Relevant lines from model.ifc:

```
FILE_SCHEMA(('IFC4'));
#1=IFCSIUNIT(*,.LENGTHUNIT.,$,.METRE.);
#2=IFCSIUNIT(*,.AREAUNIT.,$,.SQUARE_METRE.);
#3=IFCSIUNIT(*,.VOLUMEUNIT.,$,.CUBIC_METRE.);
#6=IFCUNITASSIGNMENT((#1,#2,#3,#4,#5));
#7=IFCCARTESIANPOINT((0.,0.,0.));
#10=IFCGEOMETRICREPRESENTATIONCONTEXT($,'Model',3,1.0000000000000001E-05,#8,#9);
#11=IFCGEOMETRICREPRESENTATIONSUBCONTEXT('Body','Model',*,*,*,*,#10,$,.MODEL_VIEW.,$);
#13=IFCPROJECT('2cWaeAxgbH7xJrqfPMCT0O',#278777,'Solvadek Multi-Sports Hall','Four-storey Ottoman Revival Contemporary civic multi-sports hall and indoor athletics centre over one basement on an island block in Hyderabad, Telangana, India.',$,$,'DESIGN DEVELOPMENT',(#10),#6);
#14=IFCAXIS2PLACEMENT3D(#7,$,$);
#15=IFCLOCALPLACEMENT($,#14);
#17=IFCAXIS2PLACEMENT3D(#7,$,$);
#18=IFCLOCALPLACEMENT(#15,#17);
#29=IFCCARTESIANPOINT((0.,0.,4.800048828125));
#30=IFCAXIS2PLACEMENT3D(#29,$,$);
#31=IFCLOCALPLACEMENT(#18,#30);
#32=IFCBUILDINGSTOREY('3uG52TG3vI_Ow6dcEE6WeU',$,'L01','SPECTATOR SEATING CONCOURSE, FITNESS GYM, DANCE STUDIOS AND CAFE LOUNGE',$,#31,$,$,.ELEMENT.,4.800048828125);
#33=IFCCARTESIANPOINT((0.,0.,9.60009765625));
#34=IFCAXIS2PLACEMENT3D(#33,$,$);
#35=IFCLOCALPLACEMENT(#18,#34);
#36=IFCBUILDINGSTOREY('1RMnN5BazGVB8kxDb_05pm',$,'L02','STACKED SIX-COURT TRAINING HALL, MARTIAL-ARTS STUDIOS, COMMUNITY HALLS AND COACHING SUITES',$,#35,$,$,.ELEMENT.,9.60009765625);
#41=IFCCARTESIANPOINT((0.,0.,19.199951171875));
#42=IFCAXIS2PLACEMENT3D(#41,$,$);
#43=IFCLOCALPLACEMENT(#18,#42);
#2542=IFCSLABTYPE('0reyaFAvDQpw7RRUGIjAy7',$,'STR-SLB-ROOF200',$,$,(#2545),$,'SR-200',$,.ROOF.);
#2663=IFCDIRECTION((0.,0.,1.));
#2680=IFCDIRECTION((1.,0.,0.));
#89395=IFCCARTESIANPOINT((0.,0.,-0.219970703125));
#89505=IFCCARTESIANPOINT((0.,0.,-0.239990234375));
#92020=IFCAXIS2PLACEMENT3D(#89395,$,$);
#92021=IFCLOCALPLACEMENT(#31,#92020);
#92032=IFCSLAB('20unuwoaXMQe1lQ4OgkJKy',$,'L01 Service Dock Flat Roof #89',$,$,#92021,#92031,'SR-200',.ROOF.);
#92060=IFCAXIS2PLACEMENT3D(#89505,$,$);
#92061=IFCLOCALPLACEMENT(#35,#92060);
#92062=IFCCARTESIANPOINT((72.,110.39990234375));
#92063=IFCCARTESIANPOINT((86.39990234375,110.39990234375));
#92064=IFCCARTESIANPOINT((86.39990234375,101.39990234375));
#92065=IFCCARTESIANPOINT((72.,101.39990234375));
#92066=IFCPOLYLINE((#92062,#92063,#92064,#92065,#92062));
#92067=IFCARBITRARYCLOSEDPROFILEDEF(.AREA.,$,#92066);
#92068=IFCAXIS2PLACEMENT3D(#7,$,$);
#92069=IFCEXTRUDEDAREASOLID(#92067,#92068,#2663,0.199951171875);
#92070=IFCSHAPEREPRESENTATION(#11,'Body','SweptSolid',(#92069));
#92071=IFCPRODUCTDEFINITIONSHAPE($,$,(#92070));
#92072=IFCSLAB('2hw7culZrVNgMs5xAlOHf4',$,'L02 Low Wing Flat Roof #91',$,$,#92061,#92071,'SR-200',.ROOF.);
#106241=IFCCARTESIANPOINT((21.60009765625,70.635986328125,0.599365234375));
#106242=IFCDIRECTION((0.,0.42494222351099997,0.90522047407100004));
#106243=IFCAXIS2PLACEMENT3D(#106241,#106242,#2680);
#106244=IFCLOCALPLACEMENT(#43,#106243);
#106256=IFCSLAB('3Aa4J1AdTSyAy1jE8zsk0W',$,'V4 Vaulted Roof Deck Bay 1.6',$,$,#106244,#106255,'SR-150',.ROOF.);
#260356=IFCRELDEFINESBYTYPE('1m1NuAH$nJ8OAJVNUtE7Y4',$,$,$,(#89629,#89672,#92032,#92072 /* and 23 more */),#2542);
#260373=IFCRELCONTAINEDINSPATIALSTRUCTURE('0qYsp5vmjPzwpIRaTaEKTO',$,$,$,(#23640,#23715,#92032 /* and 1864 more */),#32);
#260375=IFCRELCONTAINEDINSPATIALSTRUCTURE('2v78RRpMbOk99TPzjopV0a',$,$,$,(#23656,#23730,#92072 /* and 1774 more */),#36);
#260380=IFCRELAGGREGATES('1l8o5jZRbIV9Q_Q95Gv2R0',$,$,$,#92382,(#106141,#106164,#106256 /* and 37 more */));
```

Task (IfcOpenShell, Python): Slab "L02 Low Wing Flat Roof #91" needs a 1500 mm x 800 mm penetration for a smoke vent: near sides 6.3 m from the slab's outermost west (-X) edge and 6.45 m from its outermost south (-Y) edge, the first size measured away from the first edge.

```python
import numpy as np
import ifcopenshell
import ifcopenshell.api.feature
import ifcopenshell.api.geometry
import ifcopenshell.api.root
import ifcopenshell.geom
import ifcopenshell.util.placement
import ifcopenshell.util.representation
import ifcopenshell.util.shape
import ifcopenshell.util.unit

model = ifcopenshell.open("model.ifc")
unit_scale = ifcopenshell.util.unit.calculate_unit_scale(model)
settings = ifcopenshell.geom.settings()


def volume(element):
    """Net volume in cubic metres, openings subtracted."""
    shape = ifcopenshell.geom.create_shape(settings, element)
    return ifcopenshell.util.shape.get_volume(shape.geometry)


slab = model.by_id(92072)
before = volume(slab)

# Extent in the slab's own axes, in metres. The edges named are its -X and -Y sides.
slab_shape = ifcopenshell.geom.create_shape(settings, slab)
vertices = ifcopenshell.util.shape.get_vertices(slab_shape.geometry)
x_min, y_min, bottom = vertices.min(axis=0)
top = vertices[:, 2].max()

opening = ifcopenshell.api.root.create_entity(model, ifc_class="IfcOpeningElement", name="Smoke vent opening", predefined_type="OPENING")
context = ifcopenshell.util.representation.get_context(model, "Model", "Body", "MODEL_VIEW")
width, depth = 1.5, 0.8
outline = [(0.0, 0.0), (width, 0.0), (width, depth), (0.0, depth), (0.0, 0.0)]
# Overshoot both faces by 50 mm so the cut is clean.
shape = ifcopenshell.api.geometry.add_slab_representation(
    model, context=context, depth=top - bottom + 0.1, polyline=outline
)
ifcopenshell.api.geometry.assign_representation(model, product=opening, representation=shape)

matrix = ifcopenshell.util.placement.get_local_placement(slab.ObjectPlacement)
matrix[:, 3] = matrix @ np.append(np.array([x_min + 6.3, y_min + 6.45, bottom - 0.05]) / unit_scale, 1.0)
ifcopenshell.api.geometry.edit_object_placement(model, product=opening, matrix=matrix, is_si=False)
ifcopenshell.api.feature.add_feature(model, feature=opening, element=slab)

after = volume(slab)

print(f"slab volume {before:.3f} -> {after:.3f} m3")

model.write("model_edited.ifc")
```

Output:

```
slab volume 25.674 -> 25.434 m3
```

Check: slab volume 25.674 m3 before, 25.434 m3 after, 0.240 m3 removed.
